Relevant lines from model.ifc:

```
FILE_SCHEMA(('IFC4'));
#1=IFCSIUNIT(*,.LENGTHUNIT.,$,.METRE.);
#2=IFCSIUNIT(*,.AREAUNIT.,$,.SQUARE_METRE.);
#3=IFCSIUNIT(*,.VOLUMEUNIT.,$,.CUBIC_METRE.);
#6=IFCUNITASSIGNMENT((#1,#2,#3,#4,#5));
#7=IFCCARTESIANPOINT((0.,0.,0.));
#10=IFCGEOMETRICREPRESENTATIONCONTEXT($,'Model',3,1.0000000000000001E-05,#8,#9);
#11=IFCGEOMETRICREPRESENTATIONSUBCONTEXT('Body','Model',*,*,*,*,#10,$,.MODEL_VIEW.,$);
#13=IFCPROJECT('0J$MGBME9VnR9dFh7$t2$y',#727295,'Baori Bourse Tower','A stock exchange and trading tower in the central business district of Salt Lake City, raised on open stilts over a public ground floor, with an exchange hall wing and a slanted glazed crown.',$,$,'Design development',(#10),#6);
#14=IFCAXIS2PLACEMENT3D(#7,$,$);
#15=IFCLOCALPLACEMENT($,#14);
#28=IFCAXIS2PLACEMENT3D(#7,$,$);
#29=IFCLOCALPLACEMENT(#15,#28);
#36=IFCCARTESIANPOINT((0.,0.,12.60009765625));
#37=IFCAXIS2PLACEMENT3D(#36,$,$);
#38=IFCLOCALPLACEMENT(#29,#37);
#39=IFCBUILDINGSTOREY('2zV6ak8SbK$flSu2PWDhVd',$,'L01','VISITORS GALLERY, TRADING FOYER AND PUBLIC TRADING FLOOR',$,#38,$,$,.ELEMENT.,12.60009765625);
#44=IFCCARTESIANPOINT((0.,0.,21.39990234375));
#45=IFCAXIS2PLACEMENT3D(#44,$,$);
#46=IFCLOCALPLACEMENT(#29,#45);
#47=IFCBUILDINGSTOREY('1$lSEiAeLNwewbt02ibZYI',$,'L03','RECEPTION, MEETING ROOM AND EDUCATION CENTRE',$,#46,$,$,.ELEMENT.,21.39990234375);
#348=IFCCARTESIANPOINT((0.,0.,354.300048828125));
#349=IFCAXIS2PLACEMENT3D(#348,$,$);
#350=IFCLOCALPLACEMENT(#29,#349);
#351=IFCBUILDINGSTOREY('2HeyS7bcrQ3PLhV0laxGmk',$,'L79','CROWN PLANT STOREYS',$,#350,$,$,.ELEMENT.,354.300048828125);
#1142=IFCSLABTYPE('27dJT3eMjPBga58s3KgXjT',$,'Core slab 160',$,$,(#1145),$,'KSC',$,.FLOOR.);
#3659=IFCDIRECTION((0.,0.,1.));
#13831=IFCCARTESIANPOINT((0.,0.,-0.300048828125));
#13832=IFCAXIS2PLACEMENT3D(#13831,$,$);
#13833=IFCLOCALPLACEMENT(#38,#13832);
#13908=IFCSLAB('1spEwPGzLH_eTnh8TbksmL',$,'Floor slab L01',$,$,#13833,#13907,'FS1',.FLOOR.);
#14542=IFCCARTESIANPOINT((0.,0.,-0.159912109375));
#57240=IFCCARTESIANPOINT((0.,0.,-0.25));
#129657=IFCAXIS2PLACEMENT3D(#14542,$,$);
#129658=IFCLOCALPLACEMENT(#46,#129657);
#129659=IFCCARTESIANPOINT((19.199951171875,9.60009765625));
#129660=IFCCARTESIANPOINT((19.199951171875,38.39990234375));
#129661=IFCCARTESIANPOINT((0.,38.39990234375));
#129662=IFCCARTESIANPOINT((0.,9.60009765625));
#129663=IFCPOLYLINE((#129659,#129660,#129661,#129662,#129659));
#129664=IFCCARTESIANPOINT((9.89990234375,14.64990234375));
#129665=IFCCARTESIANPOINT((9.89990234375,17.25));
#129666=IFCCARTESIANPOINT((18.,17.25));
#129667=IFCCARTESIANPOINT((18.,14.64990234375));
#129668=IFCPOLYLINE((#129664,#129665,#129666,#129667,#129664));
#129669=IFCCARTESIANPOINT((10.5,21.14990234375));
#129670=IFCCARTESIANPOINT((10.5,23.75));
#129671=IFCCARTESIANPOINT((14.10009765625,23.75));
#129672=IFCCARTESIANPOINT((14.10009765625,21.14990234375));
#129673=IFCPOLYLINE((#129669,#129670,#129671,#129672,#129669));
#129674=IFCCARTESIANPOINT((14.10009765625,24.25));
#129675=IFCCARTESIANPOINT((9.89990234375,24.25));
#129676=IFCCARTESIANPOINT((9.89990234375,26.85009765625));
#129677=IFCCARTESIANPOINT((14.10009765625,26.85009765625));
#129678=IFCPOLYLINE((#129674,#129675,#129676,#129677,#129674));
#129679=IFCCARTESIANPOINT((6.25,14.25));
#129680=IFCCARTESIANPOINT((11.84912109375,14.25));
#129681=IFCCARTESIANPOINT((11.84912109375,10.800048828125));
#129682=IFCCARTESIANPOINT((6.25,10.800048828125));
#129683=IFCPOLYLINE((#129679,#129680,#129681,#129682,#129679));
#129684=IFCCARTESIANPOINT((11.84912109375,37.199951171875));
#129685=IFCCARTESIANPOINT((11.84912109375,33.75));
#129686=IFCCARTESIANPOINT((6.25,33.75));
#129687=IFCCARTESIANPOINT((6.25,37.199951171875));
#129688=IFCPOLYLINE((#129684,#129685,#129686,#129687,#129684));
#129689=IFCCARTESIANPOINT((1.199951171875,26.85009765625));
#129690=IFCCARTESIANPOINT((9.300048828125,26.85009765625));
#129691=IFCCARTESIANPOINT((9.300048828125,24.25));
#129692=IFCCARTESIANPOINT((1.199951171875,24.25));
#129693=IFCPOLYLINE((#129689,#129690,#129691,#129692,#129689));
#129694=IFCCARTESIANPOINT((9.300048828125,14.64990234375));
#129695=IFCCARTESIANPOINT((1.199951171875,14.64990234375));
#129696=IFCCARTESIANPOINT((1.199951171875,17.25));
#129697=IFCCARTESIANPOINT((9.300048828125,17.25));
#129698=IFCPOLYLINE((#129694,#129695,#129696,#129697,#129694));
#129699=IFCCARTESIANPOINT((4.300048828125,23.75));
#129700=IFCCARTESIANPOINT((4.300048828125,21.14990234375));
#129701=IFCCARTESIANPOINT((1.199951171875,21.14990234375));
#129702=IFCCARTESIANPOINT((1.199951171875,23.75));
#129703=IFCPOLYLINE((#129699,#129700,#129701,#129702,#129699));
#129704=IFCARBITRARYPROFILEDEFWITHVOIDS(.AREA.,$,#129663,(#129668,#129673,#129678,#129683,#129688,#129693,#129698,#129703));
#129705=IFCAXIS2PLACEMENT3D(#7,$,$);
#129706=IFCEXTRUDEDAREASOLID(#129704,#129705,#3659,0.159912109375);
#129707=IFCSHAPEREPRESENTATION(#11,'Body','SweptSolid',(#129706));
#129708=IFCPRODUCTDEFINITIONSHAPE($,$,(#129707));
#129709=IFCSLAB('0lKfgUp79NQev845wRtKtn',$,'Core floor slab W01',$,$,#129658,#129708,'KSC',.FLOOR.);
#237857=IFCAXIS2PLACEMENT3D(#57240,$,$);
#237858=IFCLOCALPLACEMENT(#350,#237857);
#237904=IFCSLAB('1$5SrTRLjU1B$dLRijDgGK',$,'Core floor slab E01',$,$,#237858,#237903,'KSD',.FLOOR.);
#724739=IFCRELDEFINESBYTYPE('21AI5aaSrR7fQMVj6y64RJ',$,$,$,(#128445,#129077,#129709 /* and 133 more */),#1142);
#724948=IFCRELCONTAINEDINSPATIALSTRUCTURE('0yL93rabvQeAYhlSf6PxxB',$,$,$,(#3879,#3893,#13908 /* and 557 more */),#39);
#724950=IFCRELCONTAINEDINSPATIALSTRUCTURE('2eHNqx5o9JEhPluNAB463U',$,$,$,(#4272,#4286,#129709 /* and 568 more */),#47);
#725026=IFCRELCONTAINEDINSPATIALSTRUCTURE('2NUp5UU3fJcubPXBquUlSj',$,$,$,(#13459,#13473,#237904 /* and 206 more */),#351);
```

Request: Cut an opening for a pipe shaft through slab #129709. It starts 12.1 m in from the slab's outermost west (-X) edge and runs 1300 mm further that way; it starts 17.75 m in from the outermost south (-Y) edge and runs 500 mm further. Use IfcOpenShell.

```python
import numpy as np
import ifcopenshell
import ifcopenshell.api.feature
import ifcopenshell.api.geometry
import ifcopenshell.api.root
import ifcopenshell.geom
import ifcopenshell.util.placement
import ifcopenshell.util.representation
import ifcopenshell.util.shape
import ifcopenshell.util.unit

model = ifcopenshell.open("model.ifc")
unit_scale = ifcopenshell.util.unit.calculate_unit_scale(model)
settings = ifcopenshell.geom.settings()


def volume(element):
    """Net volume in cubic metres, openings subtracted."""
    shape = ifcopenshell.geom.create_shape(settings, element)
    return ifcopenshell.util.shape.get_volume(shape.geometry)


slab = model.by_id(129709)
before = volume(slab)

# Extent in the slab's own axes, in metres. The edges named are its -X and -Y sides.
slab_shape = ifcopenshell.geom.create_shape(settings, slab)
vertices = ifcopenshell.util.shape.get_vertices(slab_shape.geometry)
x_min, y_min, bottom = vertices.min(axis=0)
top = vertices[:, 2].max()

opening = ifcopenshell.api.root.create_entity(model, ifc_class="IfcOpeningElement", name="Pipe shaft opening", predefined_type="OPENING")
context = ifcopenshell.util.representation.get_context(model, "Model", "Body", "MODEL_VIEW")
width, depth = 1.3, 0.5
outline = [(0.0, 0.0), (width, 0.0), (width, depth), (0.0, depth), (0.0, 0.0)]
# Overshoot both faces by 50 mm so the cut is clean.
shape = ifcopenshell.api.geometry.add_slab_representation(
    model, context=context, depth=top - bottom + 0.1, polyline=outline
)
ifcopenshell.api.geometry.assign_representation(model, product=opening, representation=shape)

matrix = ifcopenshell.util.placement.get_local_placement(slab.ObjectPlacement)
matrix[:, 3] = matrix @ np.append(np.array([x_min + 12.1, y_min + 17.75, bottom - 0.05]) / unit_scale, 1.0)
ifcopenshell.api.geometry.edit_object_placement(model, product=opening, matrix=matrix, is_si=False)
ifcopenshell.api.feature.add_feature(model, feature=opening, element=slab)

after = volume(slab)

print(f"slab volume {before:.3f} -> {after:.3f} m3")

model.write("model_edited.ifc")
```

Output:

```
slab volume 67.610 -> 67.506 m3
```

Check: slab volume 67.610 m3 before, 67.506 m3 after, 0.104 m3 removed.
